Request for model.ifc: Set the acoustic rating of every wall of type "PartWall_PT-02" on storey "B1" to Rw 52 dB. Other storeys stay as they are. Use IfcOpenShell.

First a look at what the model holds.

```python
import ifcopenshell
import ifcopenshell.util.element

model = ifcopenshell.open("model.ifc")
print(model.schema)
storey = next(s for s in model.by_type("IfcBuildingStorey") if s.Name == "B1")
walls = [e for e in ifcopenshell.util.element.get_decomposition(storey) if e.is_a("IfcWall")]
seen = {}
for e in walls:
    element_type = ifcopenshell.util.element.get_type(e)
    key = (element_type.Name if element_type != e and element_type else None, ifcopenshell.util.element.get_pset(e, "Pset_WallCommon", "AcousticRating"))
    seen[key] = seen.get(key, 0) + 1
for (name, value), count in sorted(seen.items(), key=str):
    print(count, "x", name, "|", value)
```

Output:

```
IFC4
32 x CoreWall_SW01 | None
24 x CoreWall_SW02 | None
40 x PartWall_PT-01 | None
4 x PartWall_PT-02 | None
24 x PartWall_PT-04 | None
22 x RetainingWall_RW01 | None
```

```python
import ifcopenshell
import ifcopenshell.api.pset
import ifcopenshell.util.element

model = ifcopenshell.open("model.ifc")

storey = next(s for s in model.by_type("IfcBuildingStorey") if s.Name == "B1")
walls = [e for e in ifcopenshell.util.element.get_decomposition(storey) if e.is_a("IfcWall")]

count = 0
for e in walls:
    element_type = ifcopenshell.util.element.get_type(e)
    if element_type in (None, e) or element_type.Name != "PartWall_PT-02":
        continue
    # add_pset returns the element's existing set when there is one.
    pset = ifcopenshell.api.pset.add_pset(model, product=e, name="Pset_WallCommon")
    ifcopenshell.api.pset.edit_pset(model, pset=pset, properties={"AcousticRating": "Rw 52 dB"})
    count += 1

print(count, "walls updated")

model.write("model_rev.ifc")
```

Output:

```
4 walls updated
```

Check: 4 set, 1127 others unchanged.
